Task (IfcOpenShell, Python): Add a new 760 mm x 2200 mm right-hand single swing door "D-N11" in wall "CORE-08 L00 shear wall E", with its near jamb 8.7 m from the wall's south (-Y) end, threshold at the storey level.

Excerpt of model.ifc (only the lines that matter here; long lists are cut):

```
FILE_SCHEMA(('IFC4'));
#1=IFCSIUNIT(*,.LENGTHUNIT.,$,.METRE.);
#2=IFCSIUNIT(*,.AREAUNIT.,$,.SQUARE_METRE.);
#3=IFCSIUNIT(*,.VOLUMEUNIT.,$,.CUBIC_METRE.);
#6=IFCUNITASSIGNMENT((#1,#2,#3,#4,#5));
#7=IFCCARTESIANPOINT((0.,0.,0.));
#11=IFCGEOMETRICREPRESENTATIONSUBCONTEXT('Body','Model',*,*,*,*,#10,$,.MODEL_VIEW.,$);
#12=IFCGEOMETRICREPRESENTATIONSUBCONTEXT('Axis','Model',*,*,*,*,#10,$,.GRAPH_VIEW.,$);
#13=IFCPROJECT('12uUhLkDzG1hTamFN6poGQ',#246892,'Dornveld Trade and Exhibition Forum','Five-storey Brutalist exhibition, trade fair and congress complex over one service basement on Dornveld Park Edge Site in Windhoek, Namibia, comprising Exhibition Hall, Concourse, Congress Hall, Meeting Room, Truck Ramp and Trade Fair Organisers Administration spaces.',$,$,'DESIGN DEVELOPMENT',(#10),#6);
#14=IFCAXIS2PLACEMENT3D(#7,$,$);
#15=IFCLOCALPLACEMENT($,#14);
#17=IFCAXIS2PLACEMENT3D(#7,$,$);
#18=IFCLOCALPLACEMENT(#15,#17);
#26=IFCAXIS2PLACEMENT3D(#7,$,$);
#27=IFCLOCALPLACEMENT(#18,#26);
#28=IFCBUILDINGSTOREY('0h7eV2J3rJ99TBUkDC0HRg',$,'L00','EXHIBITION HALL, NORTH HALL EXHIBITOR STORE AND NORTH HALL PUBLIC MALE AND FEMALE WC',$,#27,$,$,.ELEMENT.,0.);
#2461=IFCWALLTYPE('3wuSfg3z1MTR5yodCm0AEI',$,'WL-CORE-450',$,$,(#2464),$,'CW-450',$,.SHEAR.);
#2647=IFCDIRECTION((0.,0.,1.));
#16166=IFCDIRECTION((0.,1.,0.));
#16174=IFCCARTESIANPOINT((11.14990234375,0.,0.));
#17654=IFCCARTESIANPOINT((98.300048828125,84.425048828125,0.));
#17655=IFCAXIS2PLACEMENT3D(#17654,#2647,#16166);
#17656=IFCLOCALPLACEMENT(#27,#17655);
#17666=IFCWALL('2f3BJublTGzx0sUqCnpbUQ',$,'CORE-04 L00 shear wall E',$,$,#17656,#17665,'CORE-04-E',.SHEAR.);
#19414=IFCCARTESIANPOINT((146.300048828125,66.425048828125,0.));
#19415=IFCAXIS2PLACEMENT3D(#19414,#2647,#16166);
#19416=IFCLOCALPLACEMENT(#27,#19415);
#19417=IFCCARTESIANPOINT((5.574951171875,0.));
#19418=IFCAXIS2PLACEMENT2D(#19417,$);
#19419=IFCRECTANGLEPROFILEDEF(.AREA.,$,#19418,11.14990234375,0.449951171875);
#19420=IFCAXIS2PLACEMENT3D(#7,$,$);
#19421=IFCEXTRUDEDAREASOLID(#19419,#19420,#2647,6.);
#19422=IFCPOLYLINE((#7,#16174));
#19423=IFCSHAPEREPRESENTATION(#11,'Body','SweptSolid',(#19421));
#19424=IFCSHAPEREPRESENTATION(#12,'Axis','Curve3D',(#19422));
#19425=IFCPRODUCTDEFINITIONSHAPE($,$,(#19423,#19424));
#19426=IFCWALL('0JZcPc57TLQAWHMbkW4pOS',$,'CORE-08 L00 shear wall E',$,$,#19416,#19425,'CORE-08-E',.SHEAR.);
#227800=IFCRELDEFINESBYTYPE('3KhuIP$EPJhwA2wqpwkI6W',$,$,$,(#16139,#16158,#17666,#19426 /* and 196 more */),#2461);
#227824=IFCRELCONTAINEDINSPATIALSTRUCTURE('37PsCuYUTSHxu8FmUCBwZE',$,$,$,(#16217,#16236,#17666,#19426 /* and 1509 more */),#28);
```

```python
import numpy as np
import ifcopenshell
import ifcopenshell.api.feature
import ifcopenshell.api.geometry
import ifcopenshell.api.root
import ifcopenshell.api.spatial
import ifcopenshell.geom
import ifcopenshell.util.element
import ifcopenshell.util.placement
import ifcopenshell.util.representation
import ifcopenshell.util.shape
import ifcopenshell.util.unit

model = ifcopenshell.open("model.ifc")
unit_scale = ifcopenshell.util.unit.calculate_unit_scale(model)
settings = ifcopenshell.geom.settings()


def volume(element):
    """Net volume in cubic metres, openings subtracted."""
    shape = ifcopenshell.geom.create_shape(settings, element)
    return ifcopenshell.util.shape.get_volume(shape.geometry)


wall = model.by_guid("0JZcPc57TLQAWHMbkW4pOS")
storey = ifcopenshell.util.element.get_container(wall, ifc_class="IfcBuildingStorey")
context = ifcopenshell.util.representation.get_context(model, "Model", "Body", "MODEL_VIEW")
before = volume(wall)

width, height, from_end, sill = 0.76, 2.2, 8.7, 0.0  # metres

# The wall runs along its own X axis, and the end named is its -X end.
wall_shape = ifcopenshell.geom.create_shape(settings, wall)
x, y, z = ifcopenshell.util.shape.get_vertices(wall_shape.geometry).T
start = x.min() + from_end
face, thickness = float(y.min()), float(y.max() - y.min())
wall_matrix = ifcopenshell.util.placement.get_local_placement(wall.ObjectPlacement)
level = ifcopenshell.util.placement.get_local_placement(storey.ObjectPlacement)[2, 3]


def in_wall(x, y):
    """Placement at x, y metres in the wall's axes, at sill height."""
    matrix = wall_matrix.copy()
    matrix[:, 3] = wall_matrix @ np.array([x / unit_scale, y / unit_scale, 0.0, 1.0])
    matrix[2, 3] = level + sill / unit_scale
    return matrix


# Opening: a box that overshoots both wall faces by 50 mm.
opening = ifcopenshell.api.root.create_entity(model, ifc_class="IfcOpeningElement", predefined_type="OPENING")
box = ifcopenshell.api.geometry.add_wall_representation(
    model, context=context, length=width, height=height, thickness=thickness + 0.1
)
ifcopenshell.api.geometry.assign_representation(model, product=opening, representation=box)
ifcopenshell.api.geometry.edit_object_placement(model, product=opening, matrix=in_wall(start, face - 0.05), is_si=False)
ifcopenshell.api.feature.add_feature(model, feature=opening, element=wall)

door = ifcopenshell.api.root.create_entity(model, ifc_class="IfcDoor", name="D-N11", predefined_type="DOOR")
door.OverallWidth, door.OverallHeight = width / unit_scale, height / unit_scale
door.OperationType = "SINGLE_SWING_RIGHT"
body = ifcopenshell.api.geometry.add_door_representation(
    model,
    context=context,
    overall_width=door.OverallWidth,
    overall_height=door.OverallHeight,
    operation_type="SINGLE_SWING_RIGHT",
    lining_properties={"LiningDepth": thickness / unit_scale, "ThresholdDepth": thickness / unit_scale},
)
ifcopenshell.api.geometry.assign_representation(model, product=door, representation=body)
ifcopenshell.api.spatial.assign_container(model, products=[door], relating_structure=storey)
ifcopenshell.api.feature.add_filling(model, opening=opening, element=door)

# The lining spans the wall, so the door starts at the wall face.
ifcopenshell.api.geometry.edit_object_placement(model, product=door, matrix=in_wall(start, face), is_si=False)

after = volume(wall)

print(f"wall volume {before:.3f} -> {after:.3f} m3")

model.write("model_v2.ifc")
```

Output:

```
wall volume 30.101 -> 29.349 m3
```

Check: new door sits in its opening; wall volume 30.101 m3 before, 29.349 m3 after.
